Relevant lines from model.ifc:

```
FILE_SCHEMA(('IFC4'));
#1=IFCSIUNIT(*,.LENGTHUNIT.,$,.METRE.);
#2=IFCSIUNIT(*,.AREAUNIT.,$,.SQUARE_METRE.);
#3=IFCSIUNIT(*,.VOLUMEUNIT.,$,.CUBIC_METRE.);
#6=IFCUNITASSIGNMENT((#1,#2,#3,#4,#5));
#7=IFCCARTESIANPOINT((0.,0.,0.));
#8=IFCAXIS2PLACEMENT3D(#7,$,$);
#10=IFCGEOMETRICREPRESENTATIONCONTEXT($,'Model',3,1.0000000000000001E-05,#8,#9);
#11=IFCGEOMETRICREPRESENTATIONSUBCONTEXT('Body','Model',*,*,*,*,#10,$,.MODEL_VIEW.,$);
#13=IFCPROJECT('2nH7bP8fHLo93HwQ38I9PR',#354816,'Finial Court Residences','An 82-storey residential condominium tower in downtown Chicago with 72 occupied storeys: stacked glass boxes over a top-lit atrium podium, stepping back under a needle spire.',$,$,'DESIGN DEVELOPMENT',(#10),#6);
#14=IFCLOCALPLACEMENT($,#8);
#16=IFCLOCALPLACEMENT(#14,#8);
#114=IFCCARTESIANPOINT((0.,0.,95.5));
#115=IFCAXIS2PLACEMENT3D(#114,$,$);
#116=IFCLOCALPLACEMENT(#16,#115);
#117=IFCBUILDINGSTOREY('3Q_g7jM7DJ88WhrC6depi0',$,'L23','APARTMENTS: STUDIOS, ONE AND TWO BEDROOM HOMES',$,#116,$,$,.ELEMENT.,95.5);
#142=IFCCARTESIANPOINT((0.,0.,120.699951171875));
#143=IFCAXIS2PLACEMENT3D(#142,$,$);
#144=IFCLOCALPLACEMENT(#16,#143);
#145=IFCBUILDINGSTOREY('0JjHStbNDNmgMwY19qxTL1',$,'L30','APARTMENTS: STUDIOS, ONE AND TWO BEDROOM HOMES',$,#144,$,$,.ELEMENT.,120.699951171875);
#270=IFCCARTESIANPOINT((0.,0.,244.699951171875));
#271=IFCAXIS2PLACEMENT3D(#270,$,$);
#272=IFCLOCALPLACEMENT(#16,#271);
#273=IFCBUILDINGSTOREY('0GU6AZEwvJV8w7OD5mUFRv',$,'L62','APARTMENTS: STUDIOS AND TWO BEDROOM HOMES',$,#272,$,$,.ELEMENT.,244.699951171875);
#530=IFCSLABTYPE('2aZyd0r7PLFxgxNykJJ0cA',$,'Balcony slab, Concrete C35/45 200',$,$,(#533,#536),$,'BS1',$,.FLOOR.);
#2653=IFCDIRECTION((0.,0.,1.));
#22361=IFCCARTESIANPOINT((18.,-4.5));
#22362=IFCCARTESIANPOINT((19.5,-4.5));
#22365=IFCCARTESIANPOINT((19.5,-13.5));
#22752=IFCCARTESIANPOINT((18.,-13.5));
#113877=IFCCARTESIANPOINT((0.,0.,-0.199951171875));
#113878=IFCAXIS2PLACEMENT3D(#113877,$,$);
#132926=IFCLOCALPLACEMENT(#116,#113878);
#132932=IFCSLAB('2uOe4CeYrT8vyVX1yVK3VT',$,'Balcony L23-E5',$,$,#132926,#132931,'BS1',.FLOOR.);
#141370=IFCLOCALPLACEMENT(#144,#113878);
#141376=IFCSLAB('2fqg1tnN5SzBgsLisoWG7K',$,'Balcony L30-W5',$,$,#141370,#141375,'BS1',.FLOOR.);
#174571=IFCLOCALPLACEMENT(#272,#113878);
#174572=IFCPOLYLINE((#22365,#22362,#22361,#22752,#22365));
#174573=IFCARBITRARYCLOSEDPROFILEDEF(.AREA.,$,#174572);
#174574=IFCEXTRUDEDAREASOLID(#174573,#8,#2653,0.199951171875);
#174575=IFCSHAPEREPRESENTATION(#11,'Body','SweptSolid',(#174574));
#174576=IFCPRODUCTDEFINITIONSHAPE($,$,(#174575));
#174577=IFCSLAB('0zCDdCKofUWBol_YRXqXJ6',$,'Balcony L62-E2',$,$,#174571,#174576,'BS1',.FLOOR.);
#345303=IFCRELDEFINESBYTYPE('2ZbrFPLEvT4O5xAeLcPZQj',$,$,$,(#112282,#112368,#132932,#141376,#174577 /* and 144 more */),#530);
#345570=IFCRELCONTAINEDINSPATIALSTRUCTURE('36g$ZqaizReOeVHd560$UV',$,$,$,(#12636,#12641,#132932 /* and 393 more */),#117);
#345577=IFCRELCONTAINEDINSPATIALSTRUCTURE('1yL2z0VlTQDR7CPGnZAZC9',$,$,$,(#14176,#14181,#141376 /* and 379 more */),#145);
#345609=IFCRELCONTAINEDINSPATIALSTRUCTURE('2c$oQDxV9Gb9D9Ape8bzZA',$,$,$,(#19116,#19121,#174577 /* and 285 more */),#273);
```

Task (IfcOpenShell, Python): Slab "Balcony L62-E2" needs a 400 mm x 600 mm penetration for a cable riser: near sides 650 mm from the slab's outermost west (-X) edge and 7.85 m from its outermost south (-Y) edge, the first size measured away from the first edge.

```python
import numpy as np
import ifcopenshell
import ifcopenshell.api.feature
import ifcopenshell.api.geometry
import ifcopenshell.api.root
import ifcopenshell.geom
import ifcopenshell.util.placement
import ifcopenshell.util.representation
import ifcopenshell.util.shape
import ifcopenshell.util.unit

model = ifcopenshell.open("model.ifc")
unit_scale = ifcopenshell.util.unit.calculate_unit_scale(model)
settings = ifcopenshell.geom.settings()


def volume(element):
    """Net volume in cubic metres, openings subtracted."""
    shape = ifcopenshell.geom.create_shape(settings, element)
    return ifcopenshell.util.shape.get_volume(shape.geometry)


slab = model.by_guid("0zCDdCKofUWBol_YRXqXJ6")
before = volume(slab)

# Extent in the slab's own axes, in metres. The edges named are its -X and -Y sides.
slab_shape = ifcopenshell.geom.create_shape(settings, slab)
vertices = ifcopenshell.util.shape.get_vertices(slab_shape.geometry)
x_min, y_min, bottom = vertices.min(axis=0)
top = vertices[:, 2].max()

opening = ifcopenshell.api.root.create_entity(model, ifc_class="IfcOpeningElement", name="Cable riser opening", predefined_type="OPENING")
context = ifcopenshell.util.representation.get_context(model, "Model", "Body", "MODEL_VIEW")
width, depth = 0.4, 0.6
outline = [(0.0, 0.0), (width, 0.0), (width, depth), (0.0, depth), (0.0, 0.0)]
# Overshoot both faces by 50 mm so the cut is clean.
shape = ifcopenshell.api.geometry.add_slab_representation(
    model, context=context, depth=top - bottom + 0.1, polyline=outline
)
ifcopenshell.api.geometry.assign_representation(model, product=opening, representation=shape)

matrix = ifcopenshell.util.placement.get_local_placement(slab.ObjectPlacement)
matrix[:, 3] = matrix @ np.append(np.array([x_min + 0.65, y_min + 7.85, bottom - 0.05]) / unit_scale, 1.0)
ifcopenshell.api.geometry.edit_object_placement(model, product=opening, matrix=matrix, is_si=False)
ifcopenshell.api.feature.add_feature(model, feature=opening, element=slab)

after = volume(slab)

print(f"slab volume {before:.3f} -> {after:.3f} m3")

model.write("model_rev.ifc")
```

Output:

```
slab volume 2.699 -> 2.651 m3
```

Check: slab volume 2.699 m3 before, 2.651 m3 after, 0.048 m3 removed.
